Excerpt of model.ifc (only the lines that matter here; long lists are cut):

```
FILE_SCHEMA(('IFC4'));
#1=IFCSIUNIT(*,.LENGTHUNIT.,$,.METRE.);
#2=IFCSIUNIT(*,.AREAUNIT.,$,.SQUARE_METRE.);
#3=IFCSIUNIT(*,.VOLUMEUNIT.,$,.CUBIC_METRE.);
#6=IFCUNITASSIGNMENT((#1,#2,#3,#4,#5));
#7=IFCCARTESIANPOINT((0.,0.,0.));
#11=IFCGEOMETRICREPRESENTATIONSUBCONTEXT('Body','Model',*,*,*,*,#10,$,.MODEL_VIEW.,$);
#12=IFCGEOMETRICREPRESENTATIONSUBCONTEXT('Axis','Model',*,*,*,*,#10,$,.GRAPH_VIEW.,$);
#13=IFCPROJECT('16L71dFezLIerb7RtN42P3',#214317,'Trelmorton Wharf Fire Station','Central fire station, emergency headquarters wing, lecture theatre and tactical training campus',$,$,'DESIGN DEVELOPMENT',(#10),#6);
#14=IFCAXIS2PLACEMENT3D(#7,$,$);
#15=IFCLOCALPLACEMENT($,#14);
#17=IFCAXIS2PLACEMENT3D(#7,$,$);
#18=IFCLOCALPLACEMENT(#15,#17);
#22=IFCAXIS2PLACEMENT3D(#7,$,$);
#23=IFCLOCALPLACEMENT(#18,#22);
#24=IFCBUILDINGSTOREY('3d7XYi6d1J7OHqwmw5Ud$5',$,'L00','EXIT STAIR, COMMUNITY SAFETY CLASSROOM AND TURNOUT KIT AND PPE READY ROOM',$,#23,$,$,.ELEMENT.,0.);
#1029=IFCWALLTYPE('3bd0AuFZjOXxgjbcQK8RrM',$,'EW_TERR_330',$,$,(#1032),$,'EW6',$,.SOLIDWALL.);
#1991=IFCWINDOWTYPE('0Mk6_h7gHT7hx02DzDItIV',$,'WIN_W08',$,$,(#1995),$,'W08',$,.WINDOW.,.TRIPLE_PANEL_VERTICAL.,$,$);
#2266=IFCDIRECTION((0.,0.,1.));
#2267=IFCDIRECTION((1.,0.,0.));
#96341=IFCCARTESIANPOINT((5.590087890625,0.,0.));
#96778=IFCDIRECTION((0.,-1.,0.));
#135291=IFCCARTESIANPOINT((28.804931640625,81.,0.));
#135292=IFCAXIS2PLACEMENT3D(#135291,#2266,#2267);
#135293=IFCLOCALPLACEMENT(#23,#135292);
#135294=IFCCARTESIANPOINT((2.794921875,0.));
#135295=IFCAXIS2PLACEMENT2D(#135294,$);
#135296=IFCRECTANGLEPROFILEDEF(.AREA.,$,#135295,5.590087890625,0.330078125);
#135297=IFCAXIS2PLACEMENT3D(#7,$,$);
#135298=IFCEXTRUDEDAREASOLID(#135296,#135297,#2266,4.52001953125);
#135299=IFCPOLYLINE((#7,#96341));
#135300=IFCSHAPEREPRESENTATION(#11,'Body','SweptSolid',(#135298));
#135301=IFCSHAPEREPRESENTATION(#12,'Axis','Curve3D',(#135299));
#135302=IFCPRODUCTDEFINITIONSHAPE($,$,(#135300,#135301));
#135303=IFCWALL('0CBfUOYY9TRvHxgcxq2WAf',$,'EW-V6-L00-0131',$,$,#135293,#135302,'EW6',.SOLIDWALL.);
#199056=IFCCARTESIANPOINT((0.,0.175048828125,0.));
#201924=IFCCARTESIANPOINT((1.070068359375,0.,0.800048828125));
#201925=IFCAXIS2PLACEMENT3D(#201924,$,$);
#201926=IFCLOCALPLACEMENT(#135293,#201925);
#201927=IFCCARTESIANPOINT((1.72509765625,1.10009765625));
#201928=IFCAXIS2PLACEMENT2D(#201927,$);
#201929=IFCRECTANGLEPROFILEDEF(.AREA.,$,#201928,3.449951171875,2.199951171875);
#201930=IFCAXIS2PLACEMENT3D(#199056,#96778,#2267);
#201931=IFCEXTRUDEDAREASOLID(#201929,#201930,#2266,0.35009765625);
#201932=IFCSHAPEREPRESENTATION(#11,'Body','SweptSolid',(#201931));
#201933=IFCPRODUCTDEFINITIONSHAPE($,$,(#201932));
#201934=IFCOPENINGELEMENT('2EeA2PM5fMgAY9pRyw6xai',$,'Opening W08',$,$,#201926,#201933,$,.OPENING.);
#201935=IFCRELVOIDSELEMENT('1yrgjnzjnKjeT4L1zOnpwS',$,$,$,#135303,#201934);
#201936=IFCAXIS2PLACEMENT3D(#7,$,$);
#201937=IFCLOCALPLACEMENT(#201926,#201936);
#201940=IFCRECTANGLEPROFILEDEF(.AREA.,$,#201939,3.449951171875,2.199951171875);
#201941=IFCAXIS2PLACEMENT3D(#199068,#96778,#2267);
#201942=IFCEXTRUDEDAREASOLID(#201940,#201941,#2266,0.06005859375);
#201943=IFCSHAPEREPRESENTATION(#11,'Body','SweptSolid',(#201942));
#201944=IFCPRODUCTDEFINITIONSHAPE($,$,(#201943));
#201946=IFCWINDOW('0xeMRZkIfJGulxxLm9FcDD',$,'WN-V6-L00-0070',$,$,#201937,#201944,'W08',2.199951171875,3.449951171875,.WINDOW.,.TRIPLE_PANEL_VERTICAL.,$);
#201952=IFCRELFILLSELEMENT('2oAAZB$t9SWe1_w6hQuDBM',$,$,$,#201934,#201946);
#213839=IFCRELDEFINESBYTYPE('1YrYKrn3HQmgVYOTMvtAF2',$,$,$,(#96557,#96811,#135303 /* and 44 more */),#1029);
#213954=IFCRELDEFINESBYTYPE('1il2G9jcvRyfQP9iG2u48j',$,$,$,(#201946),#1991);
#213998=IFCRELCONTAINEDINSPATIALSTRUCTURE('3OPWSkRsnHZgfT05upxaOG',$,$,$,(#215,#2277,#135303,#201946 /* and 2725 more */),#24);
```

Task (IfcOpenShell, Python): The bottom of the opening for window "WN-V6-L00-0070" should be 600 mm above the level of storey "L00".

```python
import numpy as np
import ifcopenshell
import ifcopenshell.api.geometry
import ifcopenshell.geom
import ifcopenshell.util.element
import ifcopenshell.util.placement
import ifcopenshell.util.shape
import ifcopenshell.util.unit

model = ifcopenshell.open("model.ifc")
unit_scale = ifcopenshell.util.unit.calculate_unit_scale(model)

window = model.by_guid("0xeMRZkIfJGulxxLm9FcDD")
opening = window.FillsVoids[0].RelatingOpeningElement
storey = ifcopenshell.util.element.get_container(window, ifc_class="IfcBuildingStorey")
level = ifcopenshell.util.placement.get_local_placement(storey.ObjectPlacement)[2, 3]

# The opening's origin need not be at the sill, so measure its lowest point.
shape = ifcopenshell.geom.create_shape(ifcopenshell.geom.settings(), opening)
bottom = ifcopenshell.util.shape.get_shape_bottom_elevation(shape, shape.geometry) / unit_scale
dz = level + 0.6 - bottom

shift = np.array([0.0, 0.0, dz])
# The window is placed relative to its opening, so it follows when the opening moves.
matrix = ifcopenshell.util.placement.get_local_placement(opening.ObjectPlacement)
matrix[:3, 3] += shift
ifcopenshell.api.geometry.edit_object_placement(
    model, product=opening, matrix=matrix, is_si=False, should_transform_children=True
)

print(f"moved by {dz * unit_scale:+.3f} m")

model.write("model_rev.ifc")
```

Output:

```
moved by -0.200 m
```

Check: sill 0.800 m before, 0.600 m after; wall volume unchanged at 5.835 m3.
